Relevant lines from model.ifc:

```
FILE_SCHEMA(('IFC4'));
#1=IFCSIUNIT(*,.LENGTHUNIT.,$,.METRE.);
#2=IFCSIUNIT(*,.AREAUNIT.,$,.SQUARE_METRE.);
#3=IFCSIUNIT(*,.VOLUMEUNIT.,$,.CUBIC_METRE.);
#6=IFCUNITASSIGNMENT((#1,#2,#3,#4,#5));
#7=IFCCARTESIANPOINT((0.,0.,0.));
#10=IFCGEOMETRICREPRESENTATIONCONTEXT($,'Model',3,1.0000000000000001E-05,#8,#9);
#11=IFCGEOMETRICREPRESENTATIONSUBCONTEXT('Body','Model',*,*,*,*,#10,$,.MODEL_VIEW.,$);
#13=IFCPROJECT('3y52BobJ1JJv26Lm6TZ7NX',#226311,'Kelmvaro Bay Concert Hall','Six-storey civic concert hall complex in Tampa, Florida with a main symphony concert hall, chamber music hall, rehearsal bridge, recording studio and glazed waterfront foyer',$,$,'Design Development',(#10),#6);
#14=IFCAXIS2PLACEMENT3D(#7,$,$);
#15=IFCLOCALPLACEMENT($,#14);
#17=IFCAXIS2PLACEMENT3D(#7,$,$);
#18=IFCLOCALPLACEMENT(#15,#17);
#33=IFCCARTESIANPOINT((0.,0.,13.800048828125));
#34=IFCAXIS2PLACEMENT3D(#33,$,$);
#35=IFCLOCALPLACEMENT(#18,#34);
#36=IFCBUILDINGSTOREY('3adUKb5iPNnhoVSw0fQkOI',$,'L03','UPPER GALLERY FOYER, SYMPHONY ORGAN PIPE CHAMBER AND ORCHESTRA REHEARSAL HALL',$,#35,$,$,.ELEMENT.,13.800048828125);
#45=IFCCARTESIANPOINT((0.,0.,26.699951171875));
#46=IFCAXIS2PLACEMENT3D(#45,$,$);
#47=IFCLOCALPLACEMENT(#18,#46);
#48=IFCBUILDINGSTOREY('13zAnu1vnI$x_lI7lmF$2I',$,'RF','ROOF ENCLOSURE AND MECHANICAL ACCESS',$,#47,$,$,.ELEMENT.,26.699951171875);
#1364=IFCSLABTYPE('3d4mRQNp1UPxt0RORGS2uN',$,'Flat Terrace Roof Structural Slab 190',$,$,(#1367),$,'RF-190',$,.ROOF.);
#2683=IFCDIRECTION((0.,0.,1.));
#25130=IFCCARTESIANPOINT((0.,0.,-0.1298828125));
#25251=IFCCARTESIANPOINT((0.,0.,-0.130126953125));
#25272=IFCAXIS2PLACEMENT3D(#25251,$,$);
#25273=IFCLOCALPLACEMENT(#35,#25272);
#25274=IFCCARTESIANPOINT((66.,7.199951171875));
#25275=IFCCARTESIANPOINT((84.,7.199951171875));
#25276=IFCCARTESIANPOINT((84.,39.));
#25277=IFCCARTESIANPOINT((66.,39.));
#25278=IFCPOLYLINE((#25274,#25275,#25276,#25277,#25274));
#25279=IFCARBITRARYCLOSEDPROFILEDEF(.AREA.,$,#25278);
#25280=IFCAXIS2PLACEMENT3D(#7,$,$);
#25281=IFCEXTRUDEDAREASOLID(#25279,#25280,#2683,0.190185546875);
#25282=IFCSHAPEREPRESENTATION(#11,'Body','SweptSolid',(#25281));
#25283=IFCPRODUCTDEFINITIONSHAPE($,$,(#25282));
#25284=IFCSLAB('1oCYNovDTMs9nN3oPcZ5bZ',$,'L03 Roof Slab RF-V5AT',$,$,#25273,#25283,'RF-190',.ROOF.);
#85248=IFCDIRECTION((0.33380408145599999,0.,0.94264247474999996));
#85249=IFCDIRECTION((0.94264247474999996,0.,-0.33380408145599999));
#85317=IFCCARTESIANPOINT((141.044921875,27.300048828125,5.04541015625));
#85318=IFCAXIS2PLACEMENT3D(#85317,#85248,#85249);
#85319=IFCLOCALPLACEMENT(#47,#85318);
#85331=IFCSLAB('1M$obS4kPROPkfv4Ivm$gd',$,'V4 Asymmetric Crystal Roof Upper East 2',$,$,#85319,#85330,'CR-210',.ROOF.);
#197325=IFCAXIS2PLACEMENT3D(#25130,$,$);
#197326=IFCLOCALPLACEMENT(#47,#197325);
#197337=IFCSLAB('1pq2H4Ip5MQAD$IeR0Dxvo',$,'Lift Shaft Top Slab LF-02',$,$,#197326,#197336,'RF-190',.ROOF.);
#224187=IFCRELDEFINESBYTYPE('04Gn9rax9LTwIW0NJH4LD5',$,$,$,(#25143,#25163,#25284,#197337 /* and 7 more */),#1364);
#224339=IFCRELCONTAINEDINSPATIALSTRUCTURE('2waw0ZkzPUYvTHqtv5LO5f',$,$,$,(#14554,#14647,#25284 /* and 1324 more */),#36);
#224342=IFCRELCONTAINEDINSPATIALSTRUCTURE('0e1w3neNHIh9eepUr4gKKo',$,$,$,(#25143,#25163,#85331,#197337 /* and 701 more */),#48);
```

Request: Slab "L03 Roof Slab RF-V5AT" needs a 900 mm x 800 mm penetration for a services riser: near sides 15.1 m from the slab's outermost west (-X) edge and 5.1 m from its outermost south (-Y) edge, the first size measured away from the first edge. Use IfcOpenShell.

```python
import numpy as np
import ifcopenshell
import ifcopenshell.api.feature
import ifcopenshell.api.geometry
import ifcopenshell.api.root
import ifcopenshell.geom
import ifcopenshell.util.placement
import ifcopenshell.util.representation
import ifcopenshell.util.shape
import ifcopenshell.util.unit

model = ifcopenshell.open("model.ifc")
unit_scale = ifcopenshell.util.unit.calculate_unit_scale(model)
settings = ifcopenshell.geom.settings()


def volume(element):
    """Net volume in cubic metres, openings subtracted."""
    shape = ifcopenshell.geom.create_shape(settings, element)
    return ifcopenshell.util.shape.get_volume(shape.geometry)


slab = model.by_id(25284)
before = volume(slab)

# Extent in the slab's own axes, in metres. The edges named are its -X and -Y sides.
slab_shape = ifcopenshell.geom.create_shape(settings, slab)
vertices = ifcopenshell.util.shape.get_vertices(slab_shape.geometry)
x_min, y_min, bottom = vertices.min(axis=0)
top = vertices[:, 2].max()

opening = ifcopenshell.api.root.create_entity(model, ifc_class="IfcOpeningElement", name="Services riser opening", predefined_type="OPENING")
context = ifcopenshell.util.representation.get_context(model, "Model", "Body", "MODEL_VIEW")
width, depth = 0.9, 0.8
outline = [(0.0, 0.0), (width, 0.0), (width, depth), (0.0, depth), (0.0, 0.0)]
# Overshoot both faces by 50 mm so the cut is clean.
shape = ifcopenshell.api.geometry.add_slab_representation(
    model, context=context, depth=top - bottom + 0.1, polyline=outline
)
ifcopenshell.api.geometry.assign_representation(model, product=opening, representation=shape)

matrix = ifcopenshell.util.placement.get_local_placement(slab.ObjectPlacement)
matrix[:, 3] = matrix @ np.append(np.array([x_min + 15.1, y_min + 5.1, bottom - 0.05]) / unit_scale, 1.0)
ifcopenshell.api.geometry.edit_object_placement(model, product=opening, matrix=matrix, is_si=False)
ifcopenshell.api.feature.add_feature(model, feature=opening, element=slab)

after = volume(slab)

print(f"slab volume {before:.3f} -> {after:.3f} m3")

model.write("model_edited.ifc")
```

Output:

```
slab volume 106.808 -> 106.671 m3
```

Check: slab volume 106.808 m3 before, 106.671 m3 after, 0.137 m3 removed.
